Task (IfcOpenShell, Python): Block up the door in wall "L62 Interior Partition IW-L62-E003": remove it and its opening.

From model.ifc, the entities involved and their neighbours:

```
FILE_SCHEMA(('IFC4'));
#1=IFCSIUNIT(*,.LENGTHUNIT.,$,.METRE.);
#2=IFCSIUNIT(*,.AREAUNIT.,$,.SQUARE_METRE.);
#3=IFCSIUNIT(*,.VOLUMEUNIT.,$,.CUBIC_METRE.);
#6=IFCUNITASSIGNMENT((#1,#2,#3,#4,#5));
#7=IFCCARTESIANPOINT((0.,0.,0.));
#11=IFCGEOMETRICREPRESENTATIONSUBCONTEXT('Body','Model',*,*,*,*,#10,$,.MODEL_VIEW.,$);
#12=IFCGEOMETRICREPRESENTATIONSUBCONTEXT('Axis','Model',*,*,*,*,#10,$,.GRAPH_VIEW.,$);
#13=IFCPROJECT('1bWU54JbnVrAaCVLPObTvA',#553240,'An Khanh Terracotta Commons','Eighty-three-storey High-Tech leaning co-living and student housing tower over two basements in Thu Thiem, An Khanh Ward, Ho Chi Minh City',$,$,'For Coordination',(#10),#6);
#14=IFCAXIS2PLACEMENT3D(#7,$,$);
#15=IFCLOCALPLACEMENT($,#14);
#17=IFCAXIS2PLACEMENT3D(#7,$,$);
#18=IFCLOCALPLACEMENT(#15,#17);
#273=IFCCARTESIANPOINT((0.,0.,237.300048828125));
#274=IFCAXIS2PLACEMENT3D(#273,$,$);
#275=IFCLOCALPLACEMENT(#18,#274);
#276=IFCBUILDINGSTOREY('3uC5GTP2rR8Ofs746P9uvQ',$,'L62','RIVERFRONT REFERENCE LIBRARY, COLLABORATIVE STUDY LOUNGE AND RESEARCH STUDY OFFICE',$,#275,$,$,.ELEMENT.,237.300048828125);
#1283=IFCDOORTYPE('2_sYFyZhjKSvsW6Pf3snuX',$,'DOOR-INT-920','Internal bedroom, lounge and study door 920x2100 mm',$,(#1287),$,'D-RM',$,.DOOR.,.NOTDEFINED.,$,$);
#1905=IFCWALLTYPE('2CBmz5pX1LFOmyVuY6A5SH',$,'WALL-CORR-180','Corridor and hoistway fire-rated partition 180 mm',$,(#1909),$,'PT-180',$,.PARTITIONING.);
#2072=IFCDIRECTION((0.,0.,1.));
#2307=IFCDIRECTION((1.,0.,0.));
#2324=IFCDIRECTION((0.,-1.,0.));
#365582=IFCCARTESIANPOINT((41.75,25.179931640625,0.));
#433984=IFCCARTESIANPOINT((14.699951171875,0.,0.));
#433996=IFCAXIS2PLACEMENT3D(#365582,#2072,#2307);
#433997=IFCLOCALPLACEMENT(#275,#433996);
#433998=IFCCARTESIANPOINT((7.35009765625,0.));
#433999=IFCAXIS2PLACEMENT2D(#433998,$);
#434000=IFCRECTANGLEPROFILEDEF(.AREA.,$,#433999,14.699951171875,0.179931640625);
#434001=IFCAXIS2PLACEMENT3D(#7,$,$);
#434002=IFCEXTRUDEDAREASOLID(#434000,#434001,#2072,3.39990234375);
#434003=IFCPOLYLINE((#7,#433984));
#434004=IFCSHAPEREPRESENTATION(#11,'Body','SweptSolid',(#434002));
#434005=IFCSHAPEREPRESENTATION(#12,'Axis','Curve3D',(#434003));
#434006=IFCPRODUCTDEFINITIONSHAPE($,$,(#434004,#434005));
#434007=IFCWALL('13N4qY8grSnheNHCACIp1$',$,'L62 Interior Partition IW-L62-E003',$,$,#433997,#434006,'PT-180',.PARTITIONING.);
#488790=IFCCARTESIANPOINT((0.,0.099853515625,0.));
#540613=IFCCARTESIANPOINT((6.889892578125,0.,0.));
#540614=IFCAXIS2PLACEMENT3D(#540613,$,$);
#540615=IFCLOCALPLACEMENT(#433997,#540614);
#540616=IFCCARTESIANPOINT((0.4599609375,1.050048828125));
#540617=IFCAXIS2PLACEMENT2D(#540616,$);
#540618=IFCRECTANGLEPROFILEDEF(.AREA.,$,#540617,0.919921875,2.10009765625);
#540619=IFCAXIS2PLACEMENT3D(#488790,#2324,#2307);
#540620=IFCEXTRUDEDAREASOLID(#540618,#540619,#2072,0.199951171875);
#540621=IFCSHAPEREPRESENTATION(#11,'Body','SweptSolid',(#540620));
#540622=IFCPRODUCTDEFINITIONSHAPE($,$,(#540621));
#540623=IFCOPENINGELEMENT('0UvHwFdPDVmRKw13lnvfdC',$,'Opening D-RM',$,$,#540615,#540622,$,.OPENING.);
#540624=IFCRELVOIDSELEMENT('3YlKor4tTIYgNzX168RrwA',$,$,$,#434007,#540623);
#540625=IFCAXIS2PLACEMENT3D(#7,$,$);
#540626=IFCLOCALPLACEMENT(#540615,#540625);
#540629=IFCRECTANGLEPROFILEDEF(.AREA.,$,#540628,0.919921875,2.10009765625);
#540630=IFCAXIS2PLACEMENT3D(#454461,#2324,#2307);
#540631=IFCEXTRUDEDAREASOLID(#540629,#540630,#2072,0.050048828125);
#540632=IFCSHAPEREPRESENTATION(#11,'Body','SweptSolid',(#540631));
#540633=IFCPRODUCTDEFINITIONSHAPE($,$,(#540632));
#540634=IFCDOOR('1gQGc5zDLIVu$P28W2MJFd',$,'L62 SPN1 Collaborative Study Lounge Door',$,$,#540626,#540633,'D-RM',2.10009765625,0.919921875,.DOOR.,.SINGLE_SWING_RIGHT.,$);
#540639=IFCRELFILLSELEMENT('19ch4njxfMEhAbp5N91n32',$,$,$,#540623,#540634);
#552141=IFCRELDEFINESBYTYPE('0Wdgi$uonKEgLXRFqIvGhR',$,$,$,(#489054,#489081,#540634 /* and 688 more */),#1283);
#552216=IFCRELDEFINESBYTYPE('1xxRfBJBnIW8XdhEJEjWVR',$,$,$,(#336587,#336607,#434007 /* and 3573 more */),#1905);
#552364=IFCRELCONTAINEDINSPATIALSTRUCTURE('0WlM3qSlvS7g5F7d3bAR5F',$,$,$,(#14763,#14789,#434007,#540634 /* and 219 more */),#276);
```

```python
import ifcopenshell
import ifcopenshell.api.feature
import ifcopenshell.api.root
import ifcopenshell.geom
import ifcopenshell.util.shape

model = ifcopenshell.open("model.ifc")
settings = ifcopenshell.geom.settings()


def volume(element):
    """Net volume in cubic metres, openings subtracted."""
    shape = ifcopenshell.geom.create_shape(settings, element)
    return ifcopenshell.util.shape.get_volume(shape.geometry)


door = model.by_guid("1gQGc5zDLIVu$P28W2MJFd")
opening = door.FillsVoids[0].RelatingOpeningElement
wall = opening.VoidsElements[0].RelatingBuildingElement
before = volume(wall)

ifcopenshell.api.root.remove_product(model, product=door)
ifcopenshell.api.feature.remove_feature(model, feature=opening)

after = volume(wall)

print(f"wall volume {before:.3f} -> {after:.3f} m3")

model.write("model_updated.ifc")
```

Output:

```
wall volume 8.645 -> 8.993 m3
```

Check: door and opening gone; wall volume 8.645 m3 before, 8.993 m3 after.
